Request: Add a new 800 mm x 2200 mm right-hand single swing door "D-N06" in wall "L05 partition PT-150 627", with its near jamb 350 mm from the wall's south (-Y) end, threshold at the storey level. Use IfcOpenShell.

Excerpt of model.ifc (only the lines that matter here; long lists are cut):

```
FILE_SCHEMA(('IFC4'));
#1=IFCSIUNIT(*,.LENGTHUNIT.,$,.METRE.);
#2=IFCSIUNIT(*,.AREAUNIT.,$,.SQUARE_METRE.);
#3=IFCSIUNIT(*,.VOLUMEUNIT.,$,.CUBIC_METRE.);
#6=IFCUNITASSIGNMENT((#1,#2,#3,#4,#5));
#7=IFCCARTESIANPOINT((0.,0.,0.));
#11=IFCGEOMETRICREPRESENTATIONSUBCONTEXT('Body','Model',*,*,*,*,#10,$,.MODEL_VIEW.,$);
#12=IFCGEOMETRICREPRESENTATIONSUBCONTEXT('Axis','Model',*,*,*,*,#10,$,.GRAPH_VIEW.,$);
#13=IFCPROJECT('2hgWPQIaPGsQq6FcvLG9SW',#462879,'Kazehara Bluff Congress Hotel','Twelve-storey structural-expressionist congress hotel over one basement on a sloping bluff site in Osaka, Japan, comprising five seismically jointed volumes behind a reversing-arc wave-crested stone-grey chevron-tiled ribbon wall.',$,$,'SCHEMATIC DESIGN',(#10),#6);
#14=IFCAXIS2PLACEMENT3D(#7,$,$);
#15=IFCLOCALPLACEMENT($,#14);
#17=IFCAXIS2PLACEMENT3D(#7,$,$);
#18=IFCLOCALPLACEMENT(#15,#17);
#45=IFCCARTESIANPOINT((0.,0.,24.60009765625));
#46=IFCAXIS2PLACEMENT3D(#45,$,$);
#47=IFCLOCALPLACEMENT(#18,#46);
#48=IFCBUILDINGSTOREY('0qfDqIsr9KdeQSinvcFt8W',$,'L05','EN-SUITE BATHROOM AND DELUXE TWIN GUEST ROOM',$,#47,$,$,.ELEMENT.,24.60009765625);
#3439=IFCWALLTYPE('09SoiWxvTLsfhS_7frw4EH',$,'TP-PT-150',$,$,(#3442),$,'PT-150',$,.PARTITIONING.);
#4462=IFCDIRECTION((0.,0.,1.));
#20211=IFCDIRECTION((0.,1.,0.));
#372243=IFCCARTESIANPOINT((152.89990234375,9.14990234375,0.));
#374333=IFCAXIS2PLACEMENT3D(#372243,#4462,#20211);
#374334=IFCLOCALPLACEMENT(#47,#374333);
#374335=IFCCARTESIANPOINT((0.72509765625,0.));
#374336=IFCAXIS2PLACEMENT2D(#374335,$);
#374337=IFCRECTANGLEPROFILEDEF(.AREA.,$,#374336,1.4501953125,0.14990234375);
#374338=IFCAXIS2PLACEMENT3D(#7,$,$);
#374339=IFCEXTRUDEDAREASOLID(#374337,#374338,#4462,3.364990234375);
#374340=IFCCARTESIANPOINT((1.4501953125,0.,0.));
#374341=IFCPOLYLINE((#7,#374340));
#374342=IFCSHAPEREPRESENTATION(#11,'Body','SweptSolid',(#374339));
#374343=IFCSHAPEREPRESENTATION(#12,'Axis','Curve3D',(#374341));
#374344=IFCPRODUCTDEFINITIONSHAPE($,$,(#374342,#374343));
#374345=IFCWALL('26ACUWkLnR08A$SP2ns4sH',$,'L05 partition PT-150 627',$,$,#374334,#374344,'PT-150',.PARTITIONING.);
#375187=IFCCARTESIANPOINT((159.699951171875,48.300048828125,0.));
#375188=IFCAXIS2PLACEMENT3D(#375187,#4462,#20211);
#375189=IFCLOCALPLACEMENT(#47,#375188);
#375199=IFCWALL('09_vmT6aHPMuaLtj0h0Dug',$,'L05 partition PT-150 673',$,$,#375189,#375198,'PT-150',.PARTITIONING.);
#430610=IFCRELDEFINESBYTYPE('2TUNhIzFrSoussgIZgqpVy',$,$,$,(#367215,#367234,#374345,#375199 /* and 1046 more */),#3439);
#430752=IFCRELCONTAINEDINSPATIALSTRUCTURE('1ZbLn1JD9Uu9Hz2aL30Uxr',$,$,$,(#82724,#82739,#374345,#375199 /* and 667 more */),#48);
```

```python
import numpy as np
import ifcopenshell
import ifcopenshell.api.feature
import ifcopenshell.api.geometry
import ifcopenshell.api.root
import ifcopenshell.api.spatial
import ifcopenshell.geom
import ifcopenshell.util.element
import ifcopenshell.util.placement
import ifcopenshell.util.representation
import ifcopenshell.util.shape
import ifcopenshell.util.unit

model = ifcopenshell.open("model.ifc")
unit_scale = ifcopenshell.util.unit.calculate_unit_scale(model)
settings = ifcopenshell.geom.settings()


def volume(element):
    """Net volume in cubic metres, openings subtracted."""
    shape = ifcopenshell.geom.create_shape(settings, element)
    return ifcopenshell.util.shape.get_volume(shape.geometry)


wall = model.by_guid("26ACUWkLnR08A$SP2ns4sH")
storey = ifcopenshell.util.element.get_container(wall, ifc_class="IfcBuildingStorey")
context = ifcopenshell.util.representation.get_context(model, "Model", "Body", "MODEL_VIEW")
before = volume(wall)

width, height, from_end, sill = 0.8, 2.2, 0.35, 0.0  # metres

# The wall runs along its own X axis, and the end named is its -X end.
wall_shape = ifcopenshell.geom.create_shape(settings, wall)
x, y, z = ifcopenshell.util.shape.get_vertices(wall_shape.geometry).T
start = x.min() + from_end
face, thickness = float(y.min()), float(y.max() - y.min())
wall_matrix = ifcopenshell.util.placement.get_local_placement(wall.ObjectPlacement)
level = ifcopenshell.util.placement.get_local_placement(storey.ObjectPlacement)[2, 3]


def in_wall(x, y):
    """Placement at x, y metres in the wall's axes, at sill height."""
    matrix = wall_matrix.copy()
    matrix[:, 3] = wall_matrix @ np.array([x / unit_scale, y / unit_scale, 0.0, 1.0])
    matrix[2, 3] = level + sill / unit_scale
    return matrix


# Opening: a box that overshoots both wall faces by 50 mm.
opening = ifcopenshell.api.root.create_entity(model, ifc_class="IfcOpeningElement", predefined_type="OPENING")
box = ifcopenshell.api.geometry.add_wall_representation(
    model, context=context, length=width, height=height, thickness=thickness + 0.1
)
ifcopenshell.api.geometry.assign_representation(model, product=opening, representation=box)
ifcopenshell.api.geometry.edit_object_placement(model, product=opening, matrix=in_wall(start, face - 0.05), is_si=False)
ifcopenshell.api.feature.add_feature(model, feature=opening, element=wall)

door = ifcopenshell.api.root.create_entity(model, ifc_class="IfcDoor", name="D-N06", predefined_type="DOOR")
door.OverallWidth, door.OverallHeight = width / unit_scale, height / unit_scale
door.OperationType = "SINGLE_SWING_RIGHT"
body = ifcopenshell.api.geometry.add_door_representation(
    model,
    context=context,
    overall_width=door.OverallWidth,
    overall_height=door.OverallHeight,
    operation_type="SINGLE_SWING_RIGHT",
    lining_properties={"LiningDepth": thickness / unit_scale, "ThresholdDepth": thickness / unit_scale},
)
ifcopenshell.api.geometry.assign_representation(model, product=door, representation=body)
ifcopenshell.api.spatial.assign_container(model, products=[door], relating_structure=storey)
ifcopenshell.api.feature.add_filling(model, opening=opening, element=door)

# The lining spans the wall, so the door starts at the wall face.
ifcopenshell.api.geometry.edit_object_placement(model, product=door, matrix=in_wall(start, face), is_si=False)

after = volume(wall)

print(f"wall volume {before:.3f} -> {after:.3f} m3")

model.write("model_rev.ifc")
```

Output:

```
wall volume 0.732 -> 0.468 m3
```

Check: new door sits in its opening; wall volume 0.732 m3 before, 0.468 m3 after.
